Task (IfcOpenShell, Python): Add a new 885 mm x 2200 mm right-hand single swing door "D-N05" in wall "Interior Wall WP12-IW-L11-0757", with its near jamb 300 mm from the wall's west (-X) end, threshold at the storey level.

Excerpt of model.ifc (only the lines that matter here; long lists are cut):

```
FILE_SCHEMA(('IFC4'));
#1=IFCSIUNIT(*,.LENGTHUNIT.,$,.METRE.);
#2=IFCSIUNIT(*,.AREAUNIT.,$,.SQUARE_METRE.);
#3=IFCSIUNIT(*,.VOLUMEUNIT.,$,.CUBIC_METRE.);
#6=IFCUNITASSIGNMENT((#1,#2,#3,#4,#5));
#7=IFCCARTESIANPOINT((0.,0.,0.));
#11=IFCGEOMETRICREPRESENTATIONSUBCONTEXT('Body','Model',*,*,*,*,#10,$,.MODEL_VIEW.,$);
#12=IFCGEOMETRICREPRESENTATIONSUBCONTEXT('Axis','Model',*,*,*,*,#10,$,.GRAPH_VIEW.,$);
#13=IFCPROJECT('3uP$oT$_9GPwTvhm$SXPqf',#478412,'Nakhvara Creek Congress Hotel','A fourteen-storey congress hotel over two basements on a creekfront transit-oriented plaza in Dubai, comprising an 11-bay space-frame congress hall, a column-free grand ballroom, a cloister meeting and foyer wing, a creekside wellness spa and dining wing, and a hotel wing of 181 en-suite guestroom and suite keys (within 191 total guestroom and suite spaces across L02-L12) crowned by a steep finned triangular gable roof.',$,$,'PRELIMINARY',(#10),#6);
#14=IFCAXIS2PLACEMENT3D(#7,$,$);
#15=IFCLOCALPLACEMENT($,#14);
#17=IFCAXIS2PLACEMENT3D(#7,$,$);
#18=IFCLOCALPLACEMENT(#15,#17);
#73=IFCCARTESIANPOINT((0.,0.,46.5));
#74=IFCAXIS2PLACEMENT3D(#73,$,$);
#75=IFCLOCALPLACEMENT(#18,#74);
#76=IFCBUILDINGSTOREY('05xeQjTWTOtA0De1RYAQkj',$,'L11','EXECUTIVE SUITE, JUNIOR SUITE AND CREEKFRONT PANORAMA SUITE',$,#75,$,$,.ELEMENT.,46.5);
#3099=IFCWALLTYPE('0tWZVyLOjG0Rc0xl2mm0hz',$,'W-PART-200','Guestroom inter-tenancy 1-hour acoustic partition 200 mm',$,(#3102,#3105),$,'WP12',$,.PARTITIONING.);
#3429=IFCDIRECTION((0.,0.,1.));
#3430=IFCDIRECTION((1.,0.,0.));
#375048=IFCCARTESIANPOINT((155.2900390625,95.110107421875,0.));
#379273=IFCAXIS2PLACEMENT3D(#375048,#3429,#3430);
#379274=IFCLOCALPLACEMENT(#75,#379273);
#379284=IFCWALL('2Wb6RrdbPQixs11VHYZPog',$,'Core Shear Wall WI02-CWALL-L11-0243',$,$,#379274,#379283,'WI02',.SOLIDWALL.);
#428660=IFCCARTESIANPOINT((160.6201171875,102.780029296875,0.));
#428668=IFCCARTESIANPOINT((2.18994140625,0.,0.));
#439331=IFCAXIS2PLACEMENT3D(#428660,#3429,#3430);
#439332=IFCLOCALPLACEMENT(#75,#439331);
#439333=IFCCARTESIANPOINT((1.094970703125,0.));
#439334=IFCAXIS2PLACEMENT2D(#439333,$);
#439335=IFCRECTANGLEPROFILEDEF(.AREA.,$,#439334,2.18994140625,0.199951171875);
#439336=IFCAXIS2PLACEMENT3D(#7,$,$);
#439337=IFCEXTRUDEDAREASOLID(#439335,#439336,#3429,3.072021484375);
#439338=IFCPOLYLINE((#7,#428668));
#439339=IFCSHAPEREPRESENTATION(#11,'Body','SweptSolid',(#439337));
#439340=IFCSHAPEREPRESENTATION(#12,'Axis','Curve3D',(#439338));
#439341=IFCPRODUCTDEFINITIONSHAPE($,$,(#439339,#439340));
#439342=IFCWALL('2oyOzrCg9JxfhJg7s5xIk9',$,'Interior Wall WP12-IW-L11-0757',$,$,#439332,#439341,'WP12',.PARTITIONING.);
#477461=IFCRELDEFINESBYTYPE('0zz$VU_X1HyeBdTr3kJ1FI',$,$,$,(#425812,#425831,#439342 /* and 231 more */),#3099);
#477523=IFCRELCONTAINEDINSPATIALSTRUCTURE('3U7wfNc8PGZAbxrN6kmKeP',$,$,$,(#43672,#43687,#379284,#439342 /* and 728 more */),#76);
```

```python
import numpy as np
import ifcopenshell
import ifcopenshell.api.feature
import ifcopenshell.api.geometry
import ifcopenshell.api.root
import ifcopenshell.api.spatial
import ifcopenshell.geom
import ifcopenshell.util.element
import ifcopenshell.util.placement
import ifcopenshell.util.representation
import ifcopenshell.util.shape
import ifcopenshell.util.unit

model = ifcopenshell.open("model.ifc")
unit_scale = ifcopenshell.util.unit.calculate_unit_scale(model)
settings = ifcopenshell.geom.settings()


def volume(element):
    """Net volume in cubic metres, openings subtracted."""
    shape = ifcopenshell.geom.create_shape(settings, element)
    return ifcopenshell.util.shape.get_volume(shape.geometry)


wall = model.by_guid("2oyOzrCg9JxfhJg7s5xIk9")
storey = ifcopenshell.util.element.get_container(wall, ifc_class="IfcBuildingStorey")
context = ifcopenshell.util.representation.get_context(model, "Model", "Body", "MODEL_VIEW")
before = volume(wall)

width, height, from_end, sill = 0.885, 2.2, 0.3, 0.0  # metres

# The wall runs along its own X axis, and the end named is its -X end.
wall_shape = ifcopenshell.geom.create_shape(settings, wall)
x, y, z = ifcopenshell.util.shape.get_vertices(wall_shape.geometry).T
start = x.min() + from_end
face, thickness = float(y.min()), float(y.max() - y.min())
wall_matrix = ifcopenshell.util.placement.get_local_placement(wall.ObjectPlacement)
level = ifcopenshell.util.placement.get_local_placement(storey.ObjectPlacement)[2, 3]


def in_wall(x, y):
    """Placement at x, y metres in the wall's axes, at sill height."""
    matrix = wall_matrix.copy()
    matrix[:, 3] = wall_matrix @ np.array([x / unit_scale, y / unit_scale, 0.0, 1.0])
    matrix[2, 3] = level + sill / unit_scale
    return matrix


# Opening: a box that overshoots both wall faces by 50 mm.
opening = ifcopenshell.api.root.create_entity(model, ifc_class="IfcOpeningElement", predefined_type="OPENING")
box = ifcopenshell.api.geometry.add_wall_representation(
    model, context=context, length=width, height=height, thickness=thickness + 0.1
)
ifcopenshell.api.geometry.assign_representation(model, product=opening, representation=box)
ifcopenshell.api.geometry.edit_object_placement(model, product=opening, matrix=in_wall(start, face - 0.05), is_si=False)
ifcopenshell.api.feature.add_feature(model, feature=opening, element=wall)

door = ifcopenshell.api.root.create_entity(model, ifc_class="IfcDoor", name="D-N05", predefined_type="DOOR")
door.OverallWidth, door.OverallHeight = width / unit_scale, height / unit_scale
door.OperationType = "SINGLE_SWING_RIGHT"
body = ifcopenshell.api.geometry.add_door_representation(
    model,
    context=context,
    overall_width=door.OverallWidth,
    overall_height=door.OverallHeight,
    operation_type="SINGLE_SWING_RIGHT",
    lining_properties={"LiningDepth": thickness / unit_scale, "ThresholdDepth": thickness / unit_scale},
)
ifcopenshell.api.geometry.assign_representation(model, product=door, representation=body)
ifcopenshell.api.spatial.assign_container(model, products=[door], relating_structure=storey)
ifcopenshell.api.feature.add_filling(model, opening=opening, element=door)

# The lining spans the wall, so the door starts at the wall face.
ifcopenshell.api.geometry.edit_object_placement(model, product=door, matrix=in_wall(start, face), is_si=False)

after = volume(wall)

print(f"wall volume {before:.3f} -> {after:.3f} m3")

model.write("model_rev.ifc")
```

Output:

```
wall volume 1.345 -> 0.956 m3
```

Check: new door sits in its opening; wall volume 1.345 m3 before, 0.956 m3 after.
